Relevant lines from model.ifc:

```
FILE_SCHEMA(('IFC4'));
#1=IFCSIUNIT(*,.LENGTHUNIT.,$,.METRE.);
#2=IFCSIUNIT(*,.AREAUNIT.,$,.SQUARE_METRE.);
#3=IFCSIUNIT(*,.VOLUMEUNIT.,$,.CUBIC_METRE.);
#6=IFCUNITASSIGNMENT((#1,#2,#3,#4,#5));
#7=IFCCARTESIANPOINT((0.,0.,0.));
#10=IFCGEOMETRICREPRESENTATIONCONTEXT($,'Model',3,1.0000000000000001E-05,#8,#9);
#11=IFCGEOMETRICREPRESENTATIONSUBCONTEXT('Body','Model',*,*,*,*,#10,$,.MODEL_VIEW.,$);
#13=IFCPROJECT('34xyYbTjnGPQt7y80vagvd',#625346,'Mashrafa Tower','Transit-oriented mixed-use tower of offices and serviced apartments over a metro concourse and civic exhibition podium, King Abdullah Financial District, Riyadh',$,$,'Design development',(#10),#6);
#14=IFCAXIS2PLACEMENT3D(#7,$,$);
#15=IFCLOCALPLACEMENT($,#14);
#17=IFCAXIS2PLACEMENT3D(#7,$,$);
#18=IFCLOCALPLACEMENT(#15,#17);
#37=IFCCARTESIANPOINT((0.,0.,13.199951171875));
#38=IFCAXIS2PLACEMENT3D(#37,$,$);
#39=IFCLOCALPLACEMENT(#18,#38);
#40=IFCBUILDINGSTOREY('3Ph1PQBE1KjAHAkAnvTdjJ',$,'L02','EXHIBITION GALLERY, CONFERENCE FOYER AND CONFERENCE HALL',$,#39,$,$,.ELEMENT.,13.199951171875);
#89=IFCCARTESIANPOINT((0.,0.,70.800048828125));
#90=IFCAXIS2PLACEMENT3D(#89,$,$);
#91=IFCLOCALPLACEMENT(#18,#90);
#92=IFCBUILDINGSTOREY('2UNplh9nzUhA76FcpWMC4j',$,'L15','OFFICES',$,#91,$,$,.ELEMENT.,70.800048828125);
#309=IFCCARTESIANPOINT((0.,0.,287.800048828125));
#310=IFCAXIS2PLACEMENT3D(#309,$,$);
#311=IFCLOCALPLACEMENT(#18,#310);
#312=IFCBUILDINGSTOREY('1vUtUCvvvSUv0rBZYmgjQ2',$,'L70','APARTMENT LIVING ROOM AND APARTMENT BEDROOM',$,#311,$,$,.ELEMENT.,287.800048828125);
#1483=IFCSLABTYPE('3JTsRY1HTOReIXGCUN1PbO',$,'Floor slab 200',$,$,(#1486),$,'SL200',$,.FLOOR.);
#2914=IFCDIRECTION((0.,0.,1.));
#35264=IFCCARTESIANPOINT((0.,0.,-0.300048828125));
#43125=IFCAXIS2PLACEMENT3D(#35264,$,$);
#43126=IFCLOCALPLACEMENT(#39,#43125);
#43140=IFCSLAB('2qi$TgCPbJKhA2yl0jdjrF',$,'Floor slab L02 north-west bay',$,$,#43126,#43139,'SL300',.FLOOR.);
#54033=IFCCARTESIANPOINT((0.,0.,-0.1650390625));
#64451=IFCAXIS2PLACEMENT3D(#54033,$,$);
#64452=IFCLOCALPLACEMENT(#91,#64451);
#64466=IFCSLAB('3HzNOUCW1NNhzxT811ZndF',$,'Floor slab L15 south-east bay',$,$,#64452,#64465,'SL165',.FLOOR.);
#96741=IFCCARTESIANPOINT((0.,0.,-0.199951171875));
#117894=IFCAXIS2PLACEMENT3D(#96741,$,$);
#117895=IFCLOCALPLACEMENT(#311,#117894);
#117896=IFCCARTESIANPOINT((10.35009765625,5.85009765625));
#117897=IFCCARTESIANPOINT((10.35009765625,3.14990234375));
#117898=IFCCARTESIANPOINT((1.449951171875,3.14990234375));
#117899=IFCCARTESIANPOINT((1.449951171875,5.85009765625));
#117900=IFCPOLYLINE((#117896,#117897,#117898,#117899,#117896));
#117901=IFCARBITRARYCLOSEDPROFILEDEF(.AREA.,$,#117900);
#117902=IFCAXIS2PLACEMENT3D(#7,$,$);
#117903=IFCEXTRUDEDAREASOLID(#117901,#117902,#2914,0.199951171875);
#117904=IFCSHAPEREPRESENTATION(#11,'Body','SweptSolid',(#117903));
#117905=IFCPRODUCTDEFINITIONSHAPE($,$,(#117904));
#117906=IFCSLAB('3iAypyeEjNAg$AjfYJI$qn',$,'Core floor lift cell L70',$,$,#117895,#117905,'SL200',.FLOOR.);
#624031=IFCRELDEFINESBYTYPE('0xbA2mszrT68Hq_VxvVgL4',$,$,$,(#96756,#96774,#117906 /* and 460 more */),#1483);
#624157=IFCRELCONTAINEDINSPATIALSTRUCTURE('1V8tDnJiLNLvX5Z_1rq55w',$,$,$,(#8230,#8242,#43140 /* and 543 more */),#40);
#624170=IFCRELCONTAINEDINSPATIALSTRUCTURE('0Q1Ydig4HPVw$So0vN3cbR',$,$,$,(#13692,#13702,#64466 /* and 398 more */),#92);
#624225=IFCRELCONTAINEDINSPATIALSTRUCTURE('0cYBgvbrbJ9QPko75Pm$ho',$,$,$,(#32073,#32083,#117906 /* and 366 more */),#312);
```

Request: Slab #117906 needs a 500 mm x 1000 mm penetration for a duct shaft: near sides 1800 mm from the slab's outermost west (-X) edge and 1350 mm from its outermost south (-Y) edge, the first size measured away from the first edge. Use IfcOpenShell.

```python
import numpy as np
import ifcopenshell
import ifcopenshell.api.feature
import ifcopenshell.api.geometry
import ifcopenshell.api.root
import ifcopenshell.geom
import ifcopenshell.util.placement
import ifcopenshell.util.representation
import ifcopenshell.util.shape
import ifcopenshell.util.unit

model = ifcopenshell.open("model.ifc")
unit_scale = ifcopenshell.util.unit.calculate_unit_scale(model)
settings = ifcopenshell.geom.settings()


def volume(element):
    """Net volume in cubic metres, openings subtracted."""
    shape = ifcopenshell.geom.create_shape(settings, element)
    return ifcopenshell.util.shape.get_volume(shape.geometry)


slab = model.by_guid("3iAypyeEjNAg$AjfYJI$qn")
before = volume(slab)

# Extent in the slab's own axes, in metres. The edges named are its -X and -Y sides.
slab_shape = ifcopenshell.geom.create_shape(settings, slab)
vertices = ifcopenshell.util.shape.get_vertices(slab_shape.geometry)
x_min, y_min, bottom = vertices.min(axis=0)
top = vertices[:, 2].max()

opening = ifcopenshell.api.root.create_entity(model, ifc_class="IfcOpeningElement", name="Duct shaft opening", predefined_type="OPENING")
context = ifcopenshell.util.representation.get_context(model, "Model", "Body", "MODEL_VIEW")
width, depth = 0.5, 1
outline = [(0.0, 0.0), (width, 0.0), (width, depth), (0.0, depth), (0.0, 0.0)]
# Overshoot both faces by 50 mm so the cut is clean.
shape = ifcopenshell.api.geometry.add_slab_representation(
    model, context=context, depth=top - bottom + 0.1, polyline=outline
)
ifcopenshell.api.geometry.assign_representation(model, product=opening, representation=shape)

matrix = ifcopenshell.util.placement.get_local_placement(slab.ObjectPlacement)
matrix[:, 3] = matrix @ np.append(np.array([x_min + 1.8, y_min + 1.35, bottom - 0.05]) / unit_scale, 1.0)
ifcopenshell.api.geometry.edit_object_placement(model, product=opening, matrix=matrix, is_si=False)
ifcopenshell.api.feature.add_feature(model, feature=opening, element=slab)

after = volume(slab)

print(f"slab volume {before:.3f} -> {after:.3f} m3")

model.write("model_v2.ifc")
```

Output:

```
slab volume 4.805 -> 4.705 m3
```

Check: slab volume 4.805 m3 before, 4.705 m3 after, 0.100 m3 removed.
